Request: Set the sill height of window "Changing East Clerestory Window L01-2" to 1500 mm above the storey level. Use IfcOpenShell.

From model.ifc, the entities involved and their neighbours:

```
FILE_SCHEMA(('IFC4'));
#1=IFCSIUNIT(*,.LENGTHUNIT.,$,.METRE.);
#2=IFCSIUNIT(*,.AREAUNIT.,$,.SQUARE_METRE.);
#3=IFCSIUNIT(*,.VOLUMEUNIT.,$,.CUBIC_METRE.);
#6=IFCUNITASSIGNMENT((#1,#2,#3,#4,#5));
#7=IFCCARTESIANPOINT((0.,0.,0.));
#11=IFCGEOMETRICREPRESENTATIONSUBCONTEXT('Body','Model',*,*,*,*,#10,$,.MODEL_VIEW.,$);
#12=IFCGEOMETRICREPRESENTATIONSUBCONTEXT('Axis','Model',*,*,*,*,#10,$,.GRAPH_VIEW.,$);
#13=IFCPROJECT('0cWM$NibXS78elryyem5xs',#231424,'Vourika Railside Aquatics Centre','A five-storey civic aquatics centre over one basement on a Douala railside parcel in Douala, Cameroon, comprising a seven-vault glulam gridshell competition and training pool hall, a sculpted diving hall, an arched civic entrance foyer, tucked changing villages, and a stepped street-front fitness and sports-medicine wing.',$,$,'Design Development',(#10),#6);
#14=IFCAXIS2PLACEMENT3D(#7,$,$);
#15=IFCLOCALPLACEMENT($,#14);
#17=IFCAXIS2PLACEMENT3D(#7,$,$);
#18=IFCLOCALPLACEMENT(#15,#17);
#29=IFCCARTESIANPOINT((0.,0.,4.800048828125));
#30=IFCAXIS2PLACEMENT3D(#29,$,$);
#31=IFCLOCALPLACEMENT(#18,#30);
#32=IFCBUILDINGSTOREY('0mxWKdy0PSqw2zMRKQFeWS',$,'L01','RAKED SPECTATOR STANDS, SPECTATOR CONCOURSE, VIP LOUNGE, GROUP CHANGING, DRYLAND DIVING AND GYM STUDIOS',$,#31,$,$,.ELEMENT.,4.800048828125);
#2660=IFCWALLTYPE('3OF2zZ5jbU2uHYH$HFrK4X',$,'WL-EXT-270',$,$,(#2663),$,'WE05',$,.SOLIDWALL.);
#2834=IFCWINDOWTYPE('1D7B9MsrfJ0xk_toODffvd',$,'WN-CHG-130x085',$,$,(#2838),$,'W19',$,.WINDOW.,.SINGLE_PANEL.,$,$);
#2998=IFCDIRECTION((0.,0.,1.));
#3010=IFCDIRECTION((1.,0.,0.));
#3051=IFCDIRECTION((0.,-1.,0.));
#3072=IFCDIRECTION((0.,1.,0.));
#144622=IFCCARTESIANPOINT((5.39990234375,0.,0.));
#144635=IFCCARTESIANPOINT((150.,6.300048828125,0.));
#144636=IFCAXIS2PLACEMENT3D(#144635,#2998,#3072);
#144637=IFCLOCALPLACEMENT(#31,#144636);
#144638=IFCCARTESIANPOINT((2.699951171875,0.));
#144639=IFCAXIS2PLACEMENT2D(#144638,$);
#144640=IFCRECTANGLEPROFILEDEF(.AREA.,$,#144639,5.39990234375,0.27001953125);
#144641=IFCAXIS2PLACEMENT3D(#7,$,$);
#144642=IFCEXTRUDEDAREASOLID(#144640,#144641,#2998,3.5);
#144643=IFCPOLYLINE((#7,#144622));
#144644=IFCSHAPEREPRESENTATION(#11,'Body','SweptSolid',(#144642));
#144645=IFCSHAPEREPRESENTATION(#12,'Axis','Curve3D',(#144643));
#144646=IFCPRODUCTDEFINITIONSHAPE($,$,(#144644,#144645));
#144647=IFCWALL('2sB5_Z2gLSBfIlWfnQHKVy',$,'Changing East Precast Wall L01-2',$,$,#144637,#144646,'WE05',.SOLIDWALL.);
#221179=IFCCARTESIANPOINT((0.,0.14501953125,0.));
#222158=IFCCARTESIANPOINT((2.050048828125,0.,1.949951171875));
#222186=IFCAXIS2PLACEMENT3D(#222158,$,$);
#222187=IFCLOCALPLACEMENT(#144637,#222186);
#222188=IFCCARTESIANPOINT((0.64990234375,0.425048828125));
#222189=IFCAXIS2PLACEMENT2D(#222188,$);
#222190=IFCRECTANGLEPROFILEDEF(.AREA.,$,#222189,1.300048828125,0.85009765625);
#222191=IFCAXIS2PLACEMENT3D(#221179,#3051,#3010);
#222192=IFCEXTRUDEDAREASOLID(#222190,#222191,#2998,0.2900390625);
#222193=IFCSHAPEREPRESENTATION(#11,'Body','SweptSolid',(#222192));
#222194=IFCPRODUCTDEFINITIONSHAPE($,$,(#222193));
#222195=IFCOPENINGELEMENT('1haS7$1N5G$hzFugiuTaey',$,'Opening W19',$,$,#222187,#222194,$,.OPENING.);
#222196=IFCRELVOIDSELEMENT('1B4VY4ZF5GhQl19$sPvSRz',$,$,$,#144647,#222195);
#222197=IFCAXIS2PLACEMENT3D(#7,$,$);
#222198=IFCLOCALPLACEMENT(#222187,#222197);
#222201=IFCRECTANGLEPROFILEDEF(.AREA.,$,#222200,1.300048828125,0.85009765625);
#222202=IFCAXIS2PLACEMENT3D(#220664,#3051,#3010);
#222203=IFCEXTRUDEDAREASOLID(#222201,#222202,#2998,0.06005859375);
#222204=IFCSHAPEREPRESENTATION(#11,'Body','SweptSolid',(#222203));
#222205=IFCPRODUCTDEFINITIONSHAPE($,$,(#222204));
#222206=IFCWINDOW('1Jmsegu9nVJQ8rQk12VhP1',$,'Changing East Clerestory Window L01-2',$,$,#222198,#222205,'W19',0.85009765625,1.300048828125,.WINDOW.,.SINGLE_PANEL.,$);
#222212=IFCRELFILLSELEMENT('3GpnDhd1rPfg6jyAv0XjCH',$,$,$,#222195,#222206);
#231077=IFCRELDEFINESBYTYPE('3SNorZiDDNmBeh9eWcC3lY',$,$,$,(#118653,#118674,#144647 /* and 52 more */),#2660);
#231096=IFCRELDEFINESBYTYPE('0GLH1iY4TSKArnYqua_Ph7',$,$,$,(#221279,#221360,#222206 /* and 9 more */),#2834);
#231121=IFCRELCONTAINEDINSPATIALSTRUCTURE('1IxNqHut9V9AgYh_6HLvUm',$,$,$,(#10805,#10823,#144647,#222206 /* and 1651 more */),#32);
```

```python
import numpy as np
import ifcopenshell
import ifcopenshell.api.geometry
import ifcopenshell.geom
import ifcopenshell.util.element
import ifcopenshell.util.placement
import ifcopenshell.util.shape
import ifcopenshell.util.unit

model = ifcopenshell.open("model.ifc")
unit_scale = ifcopenshell.util.unit.calculate_unit_scale(model)

window = model.by_guid("1Jmsegu9nVJQ8rQk12VhP1")
opening = window.FillsVoids[0].RelatingOpeningElement
storey = ifcopenshell.util.element.get_container(window, ifc_class="IfcBuildingStorey")
level = ifcopenshell.util.placement.get_local_placement(storey.ObjectPlacement)[2, 3]

# The opening's origin need not be at the sill, so measure its lowest point.
shape = ifcopenshell.geom.create_shape(ifcopenshell.geom.settings(), opening)
bottom = ifcopenshell.util.shape.get_shape_bottom_elevation(shape, shape.geometry) / unit_scale
dz = level + 1.5 / unit_scale - bottom

shift = np.array([0.0, 0.0, dz])
# The window is placed relative to its opening, so it follows when the opening moves.
matrix = ifcopenshell.util.placement.get_local_placement(opening.ObjectPlacement)
matrix[:3, 3] += shift
ifcopenshell.api.geometry.edit_object_placement(
    model, product=opening, matrix=matrix, is_si=False, should_transform_children=True
)

print(f"moved by {dz * unit_scale:+.3f} m")

model.write("model_v2.ifc")
```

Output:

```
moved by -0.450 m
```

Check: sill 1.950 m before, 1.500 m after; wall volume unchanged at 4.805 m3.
